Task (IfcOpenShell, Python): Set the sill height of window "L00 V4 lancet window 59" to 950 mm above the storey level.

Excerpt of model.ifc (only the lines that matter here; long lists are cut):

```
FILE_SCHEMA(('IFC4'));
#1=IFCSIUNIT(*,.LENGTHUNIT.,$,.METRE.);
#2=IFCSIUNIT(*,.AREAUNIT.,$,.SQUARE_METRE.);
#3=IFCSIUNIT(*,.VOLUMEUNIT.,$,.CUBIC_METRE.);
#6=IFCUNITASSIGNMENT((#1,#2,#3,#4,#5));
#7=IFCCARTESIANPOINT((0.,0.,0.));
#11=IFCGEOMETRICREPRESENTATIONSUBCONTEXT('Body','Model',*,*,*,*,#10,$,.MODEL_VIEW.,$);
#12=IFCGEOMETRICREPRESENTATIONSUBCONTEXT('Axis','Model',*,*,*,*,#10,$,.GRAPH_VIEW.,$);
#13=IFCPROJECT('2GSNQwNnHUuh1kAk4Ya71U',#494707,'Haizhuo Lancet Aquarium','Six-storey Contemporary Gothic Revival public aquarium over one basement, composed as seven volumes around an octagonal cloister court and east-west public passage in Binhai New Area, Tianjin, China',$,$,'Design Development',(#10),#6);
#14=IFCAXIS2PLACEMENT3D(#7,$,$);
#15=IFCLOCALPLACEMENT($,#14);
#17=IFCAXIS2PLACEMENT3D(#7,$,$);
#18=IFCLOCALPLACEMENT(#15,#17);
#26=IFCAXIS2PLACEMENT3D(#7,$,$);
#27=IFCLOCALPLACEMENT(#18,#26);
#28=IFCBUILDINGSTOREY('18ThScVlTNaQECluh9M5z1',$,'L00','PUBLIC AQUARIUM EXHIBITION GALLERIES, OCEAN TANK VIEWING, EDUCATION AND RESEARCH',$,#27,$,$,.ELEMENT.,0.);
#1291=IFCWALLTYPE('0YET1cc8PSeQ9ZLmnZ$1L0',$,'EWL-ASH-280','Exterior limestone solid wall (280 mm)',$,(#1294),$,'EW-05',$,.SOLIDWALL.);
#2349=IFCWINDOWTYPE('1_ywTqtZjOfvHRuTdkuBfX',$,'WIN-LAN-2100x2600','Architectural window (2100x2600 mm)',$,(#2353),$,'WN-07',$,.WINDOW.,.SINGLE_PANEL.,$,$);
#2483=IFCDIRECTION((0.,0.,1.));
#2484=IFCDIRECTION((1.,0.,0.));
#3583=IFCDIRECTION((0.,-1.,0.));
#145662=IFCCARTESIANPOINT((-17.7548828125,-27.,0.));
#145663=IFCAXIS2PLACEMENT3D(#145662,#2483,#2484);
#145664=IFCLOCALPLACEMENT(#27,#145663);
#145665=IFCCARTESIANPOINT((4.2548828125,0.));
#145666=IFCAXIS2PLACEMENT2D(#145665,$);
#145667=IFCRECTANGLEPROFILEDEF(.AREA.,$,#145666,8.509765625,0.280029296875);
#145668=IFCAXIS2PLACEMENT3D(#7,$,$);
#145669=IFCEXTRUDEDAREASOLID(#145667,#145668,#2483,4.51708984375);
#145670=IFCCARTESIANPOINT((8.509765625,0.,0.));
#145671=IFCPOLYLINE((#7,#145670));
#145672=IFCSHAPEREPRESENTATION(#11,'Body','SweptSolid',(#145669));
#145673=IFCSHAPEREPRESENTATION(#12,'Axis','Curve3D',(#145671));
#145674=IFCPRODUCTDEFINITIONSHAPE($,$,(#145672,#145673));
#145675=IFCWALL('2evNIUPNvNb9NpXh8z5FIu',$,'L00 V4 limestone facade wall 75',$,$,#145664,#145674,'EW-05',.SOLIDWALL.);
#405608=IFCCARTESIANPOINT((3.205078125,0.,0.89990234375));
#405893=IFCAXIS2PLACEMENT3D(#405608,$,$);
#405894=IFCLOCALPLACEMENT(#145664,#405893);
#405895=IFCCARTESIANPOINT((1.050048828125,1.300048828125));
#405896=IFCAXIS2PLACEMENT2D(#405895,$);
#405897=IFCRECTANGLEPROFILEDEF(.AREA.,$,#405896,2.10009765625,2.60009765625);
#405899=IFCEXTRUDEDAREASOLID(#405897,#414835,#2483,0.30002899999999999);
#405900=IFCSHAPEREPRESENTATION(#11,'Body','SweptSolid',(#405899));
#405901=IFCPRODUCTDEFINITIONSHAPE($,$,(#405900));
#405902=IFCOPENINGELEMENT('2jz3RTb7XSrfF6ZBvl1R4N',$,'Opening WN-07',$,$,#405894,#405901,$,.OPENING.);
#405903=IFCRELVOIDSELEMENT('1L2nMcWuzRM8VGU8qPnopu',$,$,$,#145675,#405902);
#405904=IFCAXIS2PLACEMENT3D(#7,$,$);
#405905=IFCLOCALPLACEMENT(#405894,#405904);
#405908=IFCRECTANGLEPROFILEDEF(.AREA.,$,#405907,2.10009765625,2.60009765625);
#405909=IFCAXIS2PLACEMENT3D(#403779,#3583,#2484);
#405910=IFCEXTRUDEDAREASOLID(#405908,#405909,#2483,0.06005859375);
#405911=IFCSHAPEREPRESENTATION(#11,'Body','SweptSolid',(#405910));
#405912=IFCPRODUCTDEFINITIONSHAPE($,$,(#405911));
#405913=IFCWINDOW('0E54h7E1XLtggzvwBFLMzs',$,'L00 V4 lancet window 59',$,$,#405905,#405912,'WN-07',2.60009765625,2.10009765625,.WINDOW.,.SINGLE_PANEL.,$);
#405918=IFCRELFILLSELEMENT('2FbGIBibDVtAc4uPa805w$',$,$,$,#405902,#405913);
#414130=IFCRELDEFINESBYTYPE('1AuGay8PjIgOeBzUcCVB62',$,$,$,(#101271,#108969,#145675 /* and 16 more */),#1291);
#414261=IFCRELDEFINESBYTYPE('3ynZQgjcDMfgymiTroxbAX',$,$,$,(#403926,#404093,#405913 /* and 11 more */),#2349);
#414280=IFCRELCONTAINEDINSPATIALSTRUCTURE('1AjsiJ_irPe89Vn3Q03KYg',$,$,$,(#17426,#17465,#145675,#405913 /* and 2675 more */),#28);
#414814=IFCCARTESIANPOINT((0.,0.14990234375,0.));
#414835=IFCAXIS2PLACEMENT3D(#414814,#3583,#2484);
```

```python
import numpy as np
import ifcopenshell
import ifcopenshell.api.geometry
import ifcopenshell.geom
import ifcopenshell.util.element
import ifcopenshell.util.placement
import ifcopenshell.util.shape
import ifcopenshell.util.unit

model = ifcopenshell.open("model.ifc")
unit_scale = ifcopenshell.util.unit.calculate_unit_scale(model)

window = model.by_id(405913)
opening = window.FillsVoids[0].RelatingOpeningElement
storey = ifcopenshell.util.element.get_container(window, ifc_class="IfcBuildingStorey")
level = ifcopenshell.util.placement.get_local_placement(storey.ObjectPlacement)[2, 3]

# The opening's origin need not be at the sill, so measure its lowest point.
shape = ifcopenshell.geom.create_shape(ifcopenshell.geom.settings(), opening)
bottom = ifcopenshell.util.shape.get_shape_bottom_elevation(shape, shape.geometry) / unit_scale
dz = level + 0.95 / unit_scale - bottom

shift = np.array([0.0, 0.0, dz])
# The window is placed relative to its opening, so it follows when the opening moves.
matrix = ifcopenshell.util.placement.get_local_placement(opening.ObjectPlacement)
matrix[:3, 3] += shift
ifcopenshell.api.geometry.edit_object_placement(
    model, product=opening, matrix=matrix, is_si=False, should_transform_children=True
)

print(f"moved by {dz * unit_scale:+.3f} m")

model.write("model_updated.ifc")
```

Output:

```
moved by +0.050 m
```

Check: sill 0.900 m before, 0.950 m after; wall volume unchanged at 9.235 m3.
